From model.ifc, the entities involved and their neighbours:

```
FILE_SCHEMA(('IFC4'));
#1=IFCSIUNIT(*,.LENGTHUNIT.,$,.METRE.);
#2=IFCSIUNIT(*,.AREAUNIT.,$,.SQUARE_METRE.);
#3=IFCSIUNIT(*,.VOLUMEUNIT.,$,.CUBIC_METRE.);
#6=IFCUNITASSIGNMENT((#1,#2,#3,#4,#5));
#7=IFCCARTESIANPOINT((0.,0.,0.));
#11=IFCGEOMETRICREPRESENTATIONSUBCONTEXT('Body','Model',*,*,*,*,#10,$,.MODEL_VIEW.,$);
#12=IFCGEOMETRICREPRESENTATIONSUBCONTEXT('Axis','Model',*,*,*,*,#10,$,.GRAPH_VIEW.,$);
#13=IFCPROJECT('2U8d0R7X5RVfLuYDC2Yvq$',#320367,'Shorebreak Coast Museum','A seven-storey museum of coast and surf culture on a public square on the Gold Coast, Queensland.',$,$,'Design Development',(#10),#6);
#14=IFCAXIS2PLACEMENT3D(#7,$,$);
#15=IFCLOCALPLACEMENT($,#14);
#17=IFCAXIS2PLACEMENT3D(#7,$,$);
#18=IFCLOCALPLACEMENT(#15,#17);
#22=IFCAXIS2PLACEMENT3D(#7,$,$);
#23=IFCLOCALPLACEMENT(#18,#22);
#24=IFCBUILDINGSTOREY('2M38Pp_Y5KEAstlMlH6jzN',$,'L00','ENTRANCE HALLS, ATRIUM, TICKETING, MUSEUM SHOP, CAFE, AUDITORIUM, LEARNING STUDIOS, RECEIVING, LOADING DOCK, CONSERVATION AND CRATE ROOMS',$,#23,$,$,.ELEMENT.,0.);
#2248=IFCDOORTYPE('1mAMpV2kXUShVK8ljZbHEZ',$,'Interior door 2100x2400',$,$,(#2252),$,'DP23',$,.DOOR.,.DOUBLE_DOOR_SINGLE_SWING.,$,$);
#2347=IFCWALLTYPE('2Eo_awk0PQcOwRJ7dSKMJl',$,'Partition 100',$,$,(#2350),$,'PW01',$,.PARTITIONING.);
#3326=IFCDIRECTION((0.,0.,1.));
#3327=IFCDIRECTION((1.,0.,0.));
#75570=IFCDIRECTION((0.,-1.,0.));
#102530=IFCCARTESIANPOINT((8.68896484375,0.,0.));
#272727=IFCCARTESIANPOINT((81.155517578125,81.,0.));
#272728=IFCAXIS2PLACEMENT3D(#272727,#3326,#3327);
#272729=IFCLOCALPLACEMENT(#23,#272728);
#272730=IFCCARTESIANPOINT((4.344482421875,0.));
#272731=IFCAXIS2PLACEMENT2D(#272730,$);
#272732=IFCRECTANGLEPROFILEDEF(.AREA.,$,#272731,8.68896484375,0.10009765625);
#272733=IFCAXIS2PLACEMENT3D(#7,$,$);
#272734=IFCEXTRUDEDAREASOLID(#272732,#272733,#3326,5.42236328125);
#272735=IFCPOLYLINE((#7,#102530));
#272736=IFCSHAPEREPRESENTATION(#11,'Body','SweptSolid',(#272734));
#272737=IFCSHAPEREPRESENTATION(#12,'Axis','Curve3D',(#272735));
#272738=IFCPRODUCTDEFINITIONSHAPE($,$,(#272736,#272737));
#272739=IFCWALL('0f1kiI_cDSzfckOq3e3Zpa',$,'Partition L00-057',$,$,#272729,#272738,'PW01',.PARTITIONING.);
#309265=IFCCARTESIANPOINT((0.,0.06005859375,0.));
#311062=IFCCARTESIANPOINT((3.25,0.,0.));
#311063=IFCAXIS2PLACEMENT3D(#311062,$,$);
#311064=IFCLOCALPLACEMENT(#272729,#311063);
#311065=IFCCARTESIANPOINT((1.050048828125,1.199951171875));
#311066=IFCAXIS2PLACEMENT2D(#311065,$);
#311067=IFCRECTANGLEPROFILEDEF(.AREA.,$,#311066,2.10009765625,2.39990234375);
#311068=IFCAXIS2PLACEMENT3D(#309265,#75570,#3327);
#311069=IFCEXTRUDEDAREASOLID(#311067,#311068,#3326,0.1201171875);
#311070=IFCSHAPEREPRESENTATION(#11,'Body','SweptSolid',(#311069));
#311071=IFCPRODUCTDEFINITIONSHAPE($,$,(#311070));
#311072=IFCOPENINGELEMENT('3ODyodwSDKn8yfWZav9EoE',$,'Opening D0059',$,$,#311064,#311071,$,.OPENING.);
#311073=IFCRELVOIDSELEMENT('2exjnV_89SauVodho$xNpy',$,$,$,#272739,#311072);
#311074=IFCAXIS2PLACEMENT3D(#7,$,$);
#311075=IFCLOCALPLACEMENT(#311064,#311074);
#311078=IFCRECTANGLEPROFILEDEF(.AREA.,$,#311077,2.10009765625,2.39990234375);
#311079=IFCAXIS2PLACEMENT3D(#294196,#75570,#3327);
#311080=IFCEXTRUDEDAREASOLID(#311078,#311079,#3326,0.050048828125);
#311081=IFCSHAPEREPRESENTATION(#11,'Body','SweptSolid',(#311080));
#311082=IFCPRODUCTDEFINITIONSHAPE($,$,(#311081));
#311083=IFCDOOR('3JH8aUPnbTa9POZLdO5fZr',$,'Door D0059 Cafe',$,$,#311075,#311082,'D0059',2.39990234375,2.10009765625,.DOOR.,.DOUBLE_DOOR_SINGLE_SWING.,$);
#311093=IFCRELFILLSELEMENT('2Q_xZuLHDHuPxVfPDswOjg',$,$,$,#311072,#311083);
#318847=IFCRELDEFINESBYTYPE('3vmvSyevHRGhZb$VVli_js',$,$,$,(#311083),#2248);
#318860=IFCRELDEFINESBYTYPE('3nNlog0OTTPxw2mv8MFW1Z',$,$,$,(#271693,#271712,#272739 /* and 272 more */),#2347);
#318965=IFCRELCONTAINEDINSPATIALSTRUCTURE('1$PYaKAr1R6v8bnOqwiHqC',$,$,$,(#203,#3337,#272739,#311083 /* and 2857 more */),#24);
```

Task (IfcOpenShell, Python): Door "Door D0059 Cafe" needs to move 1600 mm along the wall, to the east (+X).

```python
import ifcopenshell
import ifcopenshell.api.geometry
import ifcopenshell.util.placement

model = ifcopenshell.open("model.ifc")

door = model.by_id(311083)
opening = door.FillsVoids[0].RelatingOpeningElement
wall = opening.VoidsElements[0].RelatingBuildingElement

wall_matrix = ifcopenshell.util.placement.get_local_placement(wall.ObjectPlacement)
shift = wall_matrix[:3, 0] * 1.6
before = ifcopenshell.util.placement.get_local_placement(door.ObjectPlacement)[:3, 3].copy()

# The door is placed relative to its opening, so it follows when the opening moves.
matrix = ifcopenshell.util.placement.get_local_placement(opening.ObjectPlacement)
matrix[:3, 3] += shift
ifcopenshell.api.geometry.edit_object_placement(
    model, product=opening, matrix=matrix, is_si=False, should_transform_children=True
)

after = ifcopenshell.util.placement.get_local_placement(door.ObjectPlacement)[:3, 3]
print("door moved by", (after - before).round(3) + 0.0)

model.write("model-out.ifc")
```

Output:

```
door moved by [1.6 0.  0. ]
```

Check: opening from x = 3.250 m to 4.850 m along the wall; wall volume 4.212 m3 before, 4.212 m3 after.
